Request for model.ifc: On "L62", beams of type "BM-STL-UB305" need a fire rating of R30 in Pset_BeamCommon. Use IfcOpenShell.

First a look at what the model holds.

```python
import ifcopenshell
import ifcopenshell.util.element

model = ifcopenshell.open("model.ifc")
print(model.schema)
storey = next(s for s in model.by_type("IfcBuildingStorey") if s.Name == "L62")
beams = [e for e in ifcopenshell.util.element.get_decomposition(storey) if e.is_a("IfcBeam")]
seen = {}
for e in beams:
    element_type = ifcopenshell.util.element.get_type(e)
    key = (element_type.Name if element_type != e and element_type else None, ifcopenshell.util.element.get_pset(e, "Pset_BeamCommon", "FireRating"))
    seen[key] = seen.get(key, 0) + 1
for (name, value), count in sorted(seen.items(), key=str):
    print(count, "x", name, "|", value)
```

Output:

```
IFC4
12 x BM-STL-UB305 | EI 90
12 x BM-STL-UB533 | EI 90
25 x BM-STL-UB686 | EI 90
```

```python
import ifcopenshell
import ifcopenshell.api.pset
import ifcopenshell.util.element

model = ifcopenshell.open("model.ifc")

storey = next(s for s in model.by_type("IfcBuildingStorey") if s.Name == "L62")
beams = [e for e in ifcopenshell.util.element.get_decomposition(storey) if e.is_a("IfcBeam")]

count = 0
for e in beams:
    element_type = ifcopenshell.util.element.get_type(e)
    if element_type in (None, e) or element_type.Name != "BM-STL-UB305":
        continue
    found = ifcopenshell.util.element.get_pset(e, "Pset_BeamCommon", should_inherit=False)
    if found:
        pset = model.by_id(found["id"])
        if len(ifcopenshell.util.element.get_elements_by_pset(pset)) > 1:
            pset = ifcopenshell.api.pset.unshare_pset(model, products=[e], pset=pset)[0]
    else:
        pset = ifcopenshell.api.pset.add_pset(model, product=e, name="Pset_BeamCommon")
    ifcopenshell.api.pset.edit_pset(model, pset=pset, properties={"FireRating": "R30"})
    count += 1

print(count, "beams updated")

model.write("model_edited.ifc")
```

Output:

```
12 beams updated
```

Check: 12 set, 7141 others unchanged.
